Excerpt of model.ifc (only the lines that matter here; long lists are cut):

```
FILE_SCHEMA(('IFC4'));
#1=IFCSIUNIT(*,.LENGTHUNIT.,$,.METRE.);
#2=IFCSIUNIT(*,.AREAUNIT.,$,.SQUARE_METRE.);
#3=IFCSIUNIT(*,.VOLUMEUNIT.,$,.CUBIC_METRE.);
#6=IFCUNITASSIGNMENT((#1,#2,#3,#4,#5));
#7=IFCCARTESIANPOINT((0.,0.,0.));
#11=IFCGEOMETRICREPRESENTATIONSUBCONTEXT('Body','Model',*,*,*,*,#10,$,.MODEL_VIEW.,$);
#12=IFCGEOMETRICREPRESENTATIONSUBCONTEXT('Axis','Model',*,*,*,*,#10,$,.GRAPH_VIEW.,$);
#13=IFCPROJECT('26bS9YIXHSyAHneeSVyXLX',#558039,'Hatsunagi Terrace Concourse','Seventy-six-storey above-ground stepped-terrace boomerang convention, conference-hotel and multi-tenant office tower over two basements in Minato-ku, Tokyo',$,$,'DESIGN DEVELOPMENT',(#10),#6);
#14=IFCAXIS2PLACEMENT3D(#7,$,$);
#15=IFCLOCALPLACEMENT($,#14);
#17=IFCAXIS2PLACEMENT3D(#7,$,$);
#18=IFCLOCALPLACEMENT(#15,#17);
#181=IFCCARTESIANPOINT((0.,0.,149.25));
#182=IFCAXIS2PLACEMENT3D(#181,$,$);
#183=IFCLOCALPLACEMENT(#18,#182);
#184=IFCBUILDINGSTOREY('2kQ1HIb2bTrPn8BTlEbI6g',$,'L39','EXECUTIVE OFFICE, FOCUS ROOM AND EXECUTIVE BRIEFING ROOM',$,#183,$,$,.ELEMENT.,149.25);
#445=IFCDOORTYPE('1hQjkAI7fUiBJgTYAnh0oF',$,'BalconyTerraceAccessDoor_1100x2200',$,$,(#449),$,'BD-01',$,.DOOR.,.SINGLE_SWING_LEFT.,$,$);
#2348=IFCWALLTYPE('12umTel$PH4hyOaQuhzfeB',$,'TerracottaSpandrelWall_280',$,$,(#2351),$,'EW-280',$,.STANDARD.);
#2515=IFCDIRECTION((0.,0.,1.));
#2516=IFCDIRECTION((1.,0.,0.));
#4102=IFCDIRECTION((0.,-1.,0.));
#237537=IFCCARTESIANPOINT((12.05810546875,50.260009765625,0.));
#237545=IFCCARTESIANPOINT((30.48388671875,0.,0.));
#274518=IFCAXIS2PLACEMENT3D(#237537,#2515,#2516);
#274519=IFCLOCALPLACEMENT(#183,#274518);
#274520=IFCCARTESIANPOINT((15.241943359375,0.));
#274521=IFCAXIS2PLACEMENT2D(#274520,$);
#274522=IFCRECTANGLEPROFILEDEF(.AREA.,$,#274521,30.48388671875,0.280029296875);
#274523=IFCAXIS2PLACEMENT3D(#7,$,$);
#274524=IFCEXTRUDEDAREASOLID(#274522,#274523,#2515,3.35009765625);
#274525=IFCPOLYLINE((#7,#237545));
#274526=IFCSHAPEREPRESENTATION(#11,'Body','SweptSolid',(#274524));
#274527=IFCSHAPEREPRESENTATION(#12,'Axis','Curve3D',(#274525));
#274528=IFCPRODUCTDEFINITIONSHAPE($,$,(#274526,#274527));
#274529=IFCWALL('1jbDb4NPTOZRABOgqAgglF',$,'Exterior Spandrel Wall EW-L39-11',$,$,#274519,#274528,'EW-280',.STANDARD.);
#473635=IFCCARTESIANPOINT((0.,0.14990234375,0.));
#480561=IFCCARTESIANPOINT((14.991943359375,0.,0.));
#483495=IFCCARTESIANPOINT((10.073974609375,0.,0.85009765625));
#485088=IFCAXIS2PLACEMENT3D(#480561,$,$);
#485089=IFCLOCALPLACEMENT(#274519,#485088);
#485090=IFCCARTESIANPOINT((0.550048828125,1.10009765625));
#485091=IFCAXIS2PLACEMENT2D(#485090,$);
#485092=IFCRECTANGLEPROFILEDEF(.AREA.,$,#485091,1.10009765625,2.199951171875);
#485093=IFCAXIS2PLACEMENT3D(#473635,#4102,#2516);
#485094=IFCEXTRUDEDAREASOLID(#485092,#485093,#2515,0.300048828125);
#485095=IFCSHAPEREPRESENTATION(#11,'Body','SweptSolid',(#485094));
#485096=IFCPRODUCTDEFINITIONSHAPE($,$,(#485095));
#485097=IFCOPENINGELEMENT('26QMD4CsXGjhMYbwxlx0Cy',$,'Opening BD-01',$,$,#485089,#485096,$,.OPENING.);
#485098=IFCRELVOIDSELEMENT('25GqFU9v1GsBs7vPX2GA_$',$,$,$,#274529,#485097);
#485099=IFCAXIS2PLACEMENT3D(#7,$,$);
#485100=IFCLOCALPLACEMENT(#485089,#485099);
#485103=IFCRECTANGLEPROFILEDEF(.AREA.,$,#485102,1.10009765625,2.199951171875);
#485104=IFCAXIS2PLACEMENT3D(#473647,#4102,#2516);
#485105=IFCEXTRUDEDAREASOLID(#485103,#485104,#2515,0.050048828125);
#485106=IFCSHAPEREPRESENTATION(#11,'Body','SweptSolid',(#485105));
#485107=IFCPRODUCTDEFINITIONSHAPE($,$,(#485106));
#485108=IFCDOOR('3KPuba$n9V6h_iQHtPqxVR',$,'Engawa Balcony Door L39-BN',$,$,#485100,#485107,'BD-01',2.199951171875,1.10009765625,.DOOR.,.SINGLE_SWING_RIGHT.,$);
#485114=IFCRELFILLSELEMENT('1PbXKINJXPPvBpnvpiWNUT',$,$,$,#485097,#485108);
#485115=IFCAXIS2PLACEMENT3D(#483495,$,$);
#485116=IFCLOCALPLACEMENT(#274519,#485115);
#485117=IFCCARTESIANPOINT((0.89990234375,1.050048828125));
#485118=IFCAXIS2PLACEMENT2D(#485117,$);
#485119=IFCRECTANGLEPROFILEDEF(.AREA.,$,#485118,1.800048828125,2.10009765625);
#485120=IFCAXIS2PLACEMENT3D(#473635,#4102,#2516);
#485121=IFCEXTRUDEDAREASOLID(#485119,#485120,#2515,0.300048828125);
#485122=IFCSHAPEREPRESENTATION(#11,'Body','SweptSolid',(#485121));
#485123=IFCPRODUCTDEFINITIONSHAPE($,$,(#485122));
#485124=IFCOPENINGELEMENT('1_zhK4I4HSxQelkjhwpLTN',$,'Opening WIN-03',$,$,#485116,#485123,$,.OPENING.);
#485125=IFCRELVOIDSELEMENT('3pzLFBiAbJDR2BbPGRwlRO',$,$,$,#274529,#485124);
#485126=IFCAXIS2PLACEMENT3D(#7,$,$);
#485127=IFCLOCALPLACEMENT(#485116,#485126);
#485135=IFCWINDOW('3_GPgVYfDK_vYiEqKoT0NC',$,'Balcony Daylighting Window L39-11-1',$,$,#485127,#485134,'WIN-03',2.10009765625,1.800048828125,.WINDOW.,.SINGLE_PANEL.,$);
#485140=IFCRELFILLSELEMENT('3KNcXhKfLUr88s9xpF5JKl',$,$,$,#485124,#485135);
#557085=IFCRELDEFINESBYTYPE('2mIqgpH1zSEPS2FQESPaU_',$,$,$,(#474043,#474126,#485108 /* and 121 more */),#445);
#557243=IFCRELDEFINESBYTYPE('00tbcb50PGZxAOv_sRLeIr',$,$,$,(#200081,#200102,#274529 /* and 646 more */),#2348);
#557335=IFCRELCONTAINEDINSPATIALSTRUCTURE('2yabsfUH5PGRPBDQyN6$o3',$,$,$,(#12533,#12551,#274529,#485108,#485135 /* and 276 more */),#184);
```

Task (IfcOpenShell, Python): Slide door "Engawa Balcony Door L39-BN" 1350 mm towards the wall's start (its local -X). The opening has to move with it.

```python
import ifcopenshell
import ifcopenshell.api.geometry
import ifcopenshell.util.placement

model = ifcopenshell.open("model.ifc")

door = model.by_id(485108)
opening = door.FillsVoids[0].RelatingOpeningElement
wall = opening.VoidsElements[0].RelatingBuildingElement

wall_matrix = ifcopenshell.util.placement.get_local_placement(wall.ObjectPlacement)
shift = wall_matrix[:3, 0] * -1.35
before = ifcopenshell.util.placement.get_local_placement(door.ObjectPlacement)[:3, 3].copy()

# The door is placed relative to its opening, so it follows when the opening moves.
matrix = ifcopenshell.util.placement.get_local_placement(opening.ObjectPlacement)
matrix[:3, 3] += shift
ifcopenshell.api.geometry.edit_object_placement(
    model, product=opening, matrix=matrix, is_si=False, should_transform_children=True
)

after = ifcopenshell.util.placement.get_local_placement(door.ObjectPlacement)[:3, 3]
print("door moved by", (after - before).round(3) + 0.0)

model.write("model_rev.ifc")
```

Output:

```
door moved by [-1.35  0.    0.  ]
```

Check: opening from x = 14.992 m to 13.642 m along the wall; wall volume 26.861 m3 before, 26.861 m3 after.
